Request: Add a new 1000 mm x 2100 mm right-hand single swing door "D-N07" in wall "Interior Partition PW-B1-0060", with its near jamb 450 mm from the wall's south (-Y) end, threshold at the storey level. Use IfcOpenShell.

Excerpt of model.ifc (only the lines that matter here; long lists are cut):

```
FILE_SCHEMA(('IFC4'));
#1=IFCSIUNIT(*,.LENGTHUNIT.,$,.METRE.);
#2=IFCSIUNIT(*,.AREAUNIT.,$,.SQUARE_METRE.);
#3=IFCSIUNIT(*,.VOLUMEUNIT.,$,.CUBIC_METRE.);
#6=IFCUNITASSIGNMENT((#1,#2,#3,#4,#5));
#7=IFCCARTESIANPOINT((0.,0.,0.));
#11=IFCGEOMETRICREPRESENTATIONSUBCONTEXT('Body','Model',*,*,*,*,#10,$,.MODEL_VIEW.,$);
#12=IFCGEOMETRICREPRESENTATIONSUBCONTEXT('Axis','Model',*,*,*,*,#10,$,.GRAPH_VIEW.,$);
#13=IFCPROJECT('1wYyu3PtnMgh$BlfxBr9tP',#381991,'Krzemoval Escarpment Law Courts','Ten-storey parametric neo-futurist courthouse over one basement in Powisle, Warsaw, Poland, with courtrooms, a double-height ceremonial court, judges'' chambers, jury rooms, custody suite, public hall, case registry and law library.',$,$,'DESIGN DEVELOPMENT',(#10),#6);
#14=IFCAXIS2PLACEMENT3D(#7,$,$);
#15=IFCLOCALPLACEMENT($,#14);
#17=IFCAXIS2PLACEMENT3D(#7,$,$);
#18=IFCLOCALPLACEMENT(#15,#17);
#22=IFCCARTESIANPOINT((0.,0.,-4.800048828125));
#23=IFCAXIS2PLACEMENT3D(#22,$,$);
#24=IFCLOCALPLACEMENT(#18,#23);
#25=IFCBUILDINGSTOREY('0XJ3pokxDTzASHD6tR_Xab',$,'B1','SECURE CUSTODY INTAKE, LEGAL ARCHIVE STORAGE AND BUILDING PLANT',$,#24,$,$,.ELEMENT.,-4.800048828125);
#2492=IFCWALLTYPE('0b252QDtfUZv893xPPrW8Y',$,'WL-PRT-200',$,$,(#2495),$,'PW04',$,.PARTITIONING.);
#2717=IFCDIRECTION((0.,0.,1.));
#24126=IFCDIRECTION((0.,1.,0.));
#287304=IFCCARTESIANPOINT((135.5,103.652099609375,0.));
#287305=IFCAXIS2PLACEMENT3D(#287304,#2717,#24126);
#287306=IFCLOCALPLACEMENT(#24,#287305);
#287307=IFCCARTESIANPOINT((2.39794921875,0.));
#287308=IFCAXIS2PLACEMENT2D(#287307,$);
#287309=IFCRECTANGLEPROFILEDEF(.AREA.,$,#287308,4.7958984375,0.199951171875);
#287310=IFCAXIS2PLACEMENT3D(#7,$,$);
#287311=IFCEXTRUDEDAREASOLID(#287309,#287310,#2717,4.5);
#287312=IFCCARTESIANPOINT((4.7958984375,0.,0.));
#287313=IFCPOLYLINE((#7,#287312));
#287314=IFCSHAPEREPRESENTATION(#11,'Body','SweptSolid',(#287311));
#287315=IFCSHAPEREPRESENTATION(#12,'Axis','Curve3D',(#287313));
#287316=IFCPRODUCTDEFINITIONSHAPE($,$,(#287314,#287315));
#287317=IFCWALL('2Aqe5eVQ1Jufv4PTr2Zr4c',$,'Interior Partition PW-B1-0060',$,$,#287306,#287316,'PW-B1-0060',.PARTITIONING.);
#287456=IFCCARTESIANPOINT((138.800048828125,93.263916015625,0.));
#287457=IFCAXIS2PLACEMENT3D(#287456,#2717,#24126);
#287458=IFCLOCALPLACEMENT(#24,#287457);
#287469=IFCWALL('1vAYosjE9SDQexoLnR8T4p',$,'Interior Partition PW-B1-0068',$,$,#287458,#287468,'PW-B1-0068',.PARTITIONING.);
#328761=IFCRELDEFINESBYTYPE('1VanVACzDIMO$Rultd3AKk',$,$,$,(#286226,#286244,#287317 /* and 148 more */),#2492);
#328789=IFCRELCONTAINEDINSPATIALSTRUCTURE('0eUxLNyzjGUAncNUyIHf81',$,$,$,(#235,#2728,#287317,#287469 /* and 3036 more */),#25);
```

```python
import numpy as np
import ifcopenshell
import ifcopenshell.api.feature
import ifcopenshell.api.geometry
import ifcopenshell.api.root
import ifcopenshell.api.spatial
import ifcopenshell.geom
import ifcopenshell.util.element
import ifcopenshell.util.placement
import ifcopenshell.util.representation
import ifcopenshell.util.shape
import ifcopenshell.util.unit

model = ifcopenshell.open("model.ifc")
unit_scale = ifcopenshell.util.unit.calculate_unit_scale(model)
settings = ifcopenshell.geom.settings()


def volume(element):
    """Net volume in cubic metres, openings subtracted."""
    shape = ifcopenshell.geom.create_shape(settings, element)
    return ifcopenshell.util.shape.get_volume(shape.geometry)


wall = model.by_id(287317)
storey = ifcopenshell.util.element.get_container(wall, ifc_class="IfcBuildingStorey")
context = ifcopenshell.util.representation.get_context(model, "Model", "Body", "MODEL_VIEW")
before = volume(wall)

width, height, from_end, sill = 1, 2.1, 0.45, 0.0  # metres

# The wall runs along its own X axis, and the end named is its -X end.
wall_shape = ifcopenshell.geom.create_shape(settings, wall)
x, y, z = ifcopenshell.util.shape.get_vertices(wall_shape.geometry).T
start = x.min() + from_end
face, thickness = float(y.min()), float(y.max() - y.min())
wall_matrix = ifcopenshell.util.placement.get_local_placement(wall.ObjectPlacement)
level = ifcopenshell.util.placement.get_local_placement(storey.ObjectPlacement)[2, 3]


def in_wall(x, y):
    """Placement at x, y metres in the wall's axes, at sill height."""
    matrix = wall_matrix.copy()
    matrix[:, 3] = wall_matrix @ np.array([x / unit_scale, y / unit_scale, 0.0, 1.0])
    matrix[2, 3] = level + sill / unit_scale
    return matrix


# Opening: a box that overshoots both wall faces by 50 mm.
opening = ifcopenshell.api.root.create_entity(model, ifc_class="IfcOpeningElement", predefined_type="OPENING")
box = ifcopenshell.api.geometry.add_wall_representation(
    model, context=context, length=width, height=height, thickness=thickness + 0.1
)
ifcopenshell.api.geometry.assign_representation(model, product=opening, representation=box)
ifcopenshell.api.geometry.edit_object_placement(model, product=opening, matrix=in_wall(start, face - 0.05), is_si=False)
ifcopenshell.api.feature.add_feature(model, feature=opening, element=wall)

door = ifcopenshell.api.root.create_entity(model, ifc_class="IfcDoor", name="D-N07", predefined_type="DOOR")
door.OverallWidth, door.OverallHeight = width / unit_scale, height / unit_scale
door.OperationType = "SINGLE_SWING_RIGHT"
body = ifcopenshell.api.geometry.add_door_representation(
    model,
    context=context,
    overall_width=door.OverallWidth,
    overall_height=door.OverallHeight,
    operation_type="SINGLE_SWING_RIGHT",
    lining_properties={"LiningDepth": thickness / unit_scale, "ThresholdDepth": thickness / unit_scale},
)
ifcopenshell.api.geometry.assign_representation(model, product=door, representation=body)
ifcopenshell.api.spatial.assign_container(model, products=[door], relating_structure=storey)
ifcopenshell.api.feature.add_filling(model, opening=opening, element=door)

# The lining spans the wall, so the door starts at the wall face.
ifcopenshell.api.geometry.edit_object_placement(model, product=door, matrix=in_wall(start, face), is_si=False)

after = volume(wall)

print(f"wall volume {before:.3f} -> {after:.3f} m3")

model.write("model_edited.ifc")
```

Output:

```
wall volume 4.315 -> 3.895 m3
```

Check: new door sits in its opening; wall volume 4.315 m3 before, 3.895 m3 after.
